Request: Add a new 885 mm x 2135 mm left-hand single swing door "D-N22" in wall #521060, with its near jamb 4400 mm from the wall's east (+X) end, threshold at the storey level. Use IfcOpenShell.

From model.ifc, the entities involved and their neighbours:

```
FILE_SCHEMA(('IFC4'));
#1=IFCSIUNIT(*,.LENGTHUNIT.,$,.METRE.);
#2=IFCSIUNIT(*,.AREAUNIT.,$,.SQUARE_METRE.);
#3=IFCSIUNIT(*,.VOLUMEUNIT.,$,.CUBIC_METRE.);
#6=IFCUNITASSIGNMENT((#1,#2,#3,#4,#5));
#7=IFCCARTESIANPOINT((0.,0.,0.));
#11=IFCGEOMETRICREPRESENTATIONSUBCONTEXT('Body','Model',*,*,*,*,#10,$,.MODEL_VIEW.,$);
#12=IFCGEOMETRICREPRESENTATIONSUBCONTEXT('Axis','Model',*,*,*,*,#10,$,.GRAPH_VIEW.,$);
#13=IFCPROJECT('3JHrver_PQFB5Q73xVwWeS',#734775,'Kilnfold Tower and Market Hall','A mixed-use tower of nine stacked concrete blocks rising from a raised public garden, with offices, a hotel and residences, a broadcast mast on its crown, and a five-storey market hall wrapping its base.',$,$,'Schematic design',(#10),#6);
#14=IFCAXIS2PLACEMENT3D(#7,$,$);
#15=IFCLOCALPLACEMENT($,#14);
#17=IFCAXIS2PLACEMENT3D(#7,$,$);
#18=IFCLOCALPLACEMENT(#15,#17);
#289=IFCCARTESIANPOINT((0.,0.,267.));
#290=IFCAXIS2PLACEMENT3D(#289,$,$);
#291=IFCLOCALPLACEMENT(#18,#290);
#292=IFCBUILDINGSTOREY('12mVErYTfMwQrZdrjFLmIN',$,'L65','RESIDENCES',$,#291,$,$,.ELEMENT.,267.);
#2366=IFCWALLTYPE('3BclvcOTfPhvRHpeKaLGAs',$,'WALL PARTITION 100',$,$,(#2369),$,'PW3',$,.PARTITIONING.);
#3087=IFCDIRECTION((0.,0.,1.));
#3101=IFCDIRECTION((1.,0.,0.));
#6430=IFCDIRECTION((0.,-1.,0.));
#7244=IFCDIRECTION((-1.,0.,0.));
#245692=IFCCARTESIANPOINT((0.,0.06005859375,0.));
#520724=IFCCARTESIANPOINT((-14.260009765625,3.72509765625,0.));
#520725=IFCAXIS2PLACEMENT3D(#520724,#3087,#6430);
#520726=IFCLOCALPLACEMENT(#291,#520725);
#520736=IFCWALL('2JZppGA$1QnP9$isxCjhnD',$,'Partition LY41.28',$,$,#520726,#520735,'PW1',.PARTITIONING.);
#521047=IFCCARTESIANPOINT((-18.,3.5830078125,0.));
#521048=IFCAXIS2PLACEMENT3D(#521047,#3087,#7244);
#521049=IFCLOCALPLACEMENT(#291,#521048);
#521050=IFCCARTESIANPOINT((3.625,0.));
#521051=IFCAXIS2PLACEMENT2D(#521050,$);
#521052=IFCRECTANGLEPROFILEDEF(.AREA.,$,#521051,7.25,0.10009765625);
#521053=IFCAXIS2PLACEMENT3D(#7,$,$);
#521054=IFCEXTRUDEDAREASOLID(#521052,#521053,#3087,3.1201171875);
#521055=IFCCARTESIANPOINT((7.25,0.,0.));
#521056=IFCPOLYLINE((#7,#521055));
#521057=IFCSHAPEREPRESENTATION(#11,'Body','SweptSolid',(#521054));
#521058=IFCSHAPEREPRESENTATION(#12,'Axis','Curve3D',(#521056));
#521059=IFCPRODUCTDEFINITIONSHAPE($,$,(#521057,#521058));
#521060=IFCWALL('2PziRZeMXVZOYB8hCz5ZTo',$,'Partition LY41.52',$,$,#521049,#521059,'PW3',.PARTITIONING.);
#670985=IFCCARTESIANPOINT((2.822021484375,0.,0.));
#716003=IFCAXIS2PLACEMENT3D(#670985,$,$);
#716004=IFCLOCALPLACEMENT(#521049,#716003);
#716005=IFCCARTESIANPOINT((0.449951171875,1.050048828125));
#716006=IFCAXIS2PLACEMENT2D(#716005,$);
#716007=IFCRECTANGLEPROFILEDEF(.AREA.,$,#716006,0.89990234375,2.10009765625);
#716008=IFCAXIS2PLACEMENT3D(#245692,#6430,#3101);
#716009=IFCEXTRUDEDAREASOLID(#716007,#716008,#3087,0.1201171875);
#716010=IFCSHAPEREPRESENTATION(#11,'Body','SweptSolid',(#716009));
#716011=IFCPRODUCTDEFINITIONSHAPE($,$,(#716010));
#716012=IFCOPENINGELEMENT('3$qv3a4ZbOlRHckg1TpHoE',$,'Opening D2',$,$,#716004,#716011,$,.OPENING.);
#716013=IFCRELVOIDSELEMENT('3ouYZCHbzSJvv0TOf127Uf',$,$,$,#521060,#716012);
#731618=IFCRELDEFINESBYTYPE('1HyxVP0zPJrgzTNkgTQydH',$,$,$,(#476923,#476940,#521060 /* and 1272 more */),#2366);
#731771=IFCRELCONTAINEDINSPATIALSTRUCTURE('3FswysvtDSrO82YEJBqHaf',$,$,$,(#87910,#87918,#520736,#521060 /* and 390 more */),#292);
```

```python
import numpy as np
import ifcopenshell
import ifcopenshell.api.feature
import ifcopenshell.api.geometry
import ifcopenshell.api.root
import ifcopenshell.api.spatial
import ifcopenshell.geom
import ifcopenshell.util.element
import ifcopenshell.util.placement
import ifcopenshell.util.representation
import ifcopenshell.util.shape
import ifcopenshell.util.unit

model = ifcopenshell.open("model.ifc")
unit_scale = ifcopenshell.util.unit.calculate_unit_scale(model)
settings = ifcopenshell.geom.settings()


def volume(element):
    """Net volume in cubic metres, openings subtracted."""
    shape = ifcopenshell.geom.create_shape(settings, element)
    return ifcopenshell.util.shape.get_volume(shape.geometry)


wall = model.by_id(521060)
storey = ifcopenshell.util.element.get_container(wall, ifc_class="IfcBuildingStorey")
context = ifcopenshell.util.representation.get_context(model, "Model", "Body", "MODEL_VIEW")
before = volume(wall)

width, height, from_end, sill = 0.885, 2.135, 4.4, 0.0  # metres

# The wall runs along its own X axis, and the end named is its -X end.
wall_shape = ifcopenshell.geom.create_shape(settings, wall)
x, y, z = ifcopenshell.util.shape.get_vertices(wall_shape.geometry).T
start = x.min() + from_end
face, thickness = float(y.min()), float(y.max() - y.min())
wall_matrix = ifcopenshell.util.placement.get_local_placement(wall.ObjectPlacement)
level = ifcopenshell.util.placement.get_local_placement(storey.ObjectPlacement)[2, 3]


def in_wall(x, y):
    """Placement at x, y metres in the wall's axes, at sill height."""
    matrix = wall_matrix.copy()
    matrix[:, 3] = wall_matrix @ np.array([x / unit_scale, y / unit_scale, 0.0, 1.0])
    matrix[2, 3] = level + sill / unit_scale
    return matrix


# Opening: a box that overshoots both wall faces by 50 mm.
opening = ifcopenshell.api.root.create_entity(model, ifc_class="IfcOpeningElement", predefined_type="OPENING")
box = ifcopenshell.api.geometry.add_wall_representation(
    model, context=context, length=width, height=height, thickness=thickness + 0.1
)
ifcopenshell.api.geometry.assign_representation(model, product=opening, representation=box)
ifcopenshell.api.geometry.edit_object_placement(model, product=opening, matrix=in_wall(start, face - 0.05), is_si=False)
ifcopenshell.api.feature.add_feature(model, feature=opening, element=wall)

door = ifcopenshell.api.root.create_entity(model, ifc_class="IfcDoor", name="D-N22", predefined_type="DOOR")
door.OverallWidth, door.OverallHeight = width / unit_scale, height / unit_scale
door.OperationType = "SINGLE_SWING_LEFT"
body = ifcopenshell.api.geometry.add_door_representation(
    model,
    context=context,
    overall_width=door.OverallWidth,
    overall_height=door.OverallHeight,
    operation_type="SINGLE_SWING_LEFT",
    lining_properties={"LiningDepth": thickness / unit_scale, "ThresholdDepth": thickness / unit_scale},
)
ifcopenshell.api.geometry.assign_representation(model, product=door, representation=body)
ifcopenshell.api.spatial.assign_container(model, products=[door], relating_structure=storey)
ifcopenshell.api.feature.add_filling(model, opening=opening, element=door)

# The lining spans the wall, so the door starts at the wall face.
ifcopenshell.api.geometry.edit_object_placement(model, product=door, matrix=in_wall(start, face), is_si=False)

after = volume(wall)

print(f"wall volume {before:.3f} -> {after:.3f} m3")

model.write("model_updated.ifc")
```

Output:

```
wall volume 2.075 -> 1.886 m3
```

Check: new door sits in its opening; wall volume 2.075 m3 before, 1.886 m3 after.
